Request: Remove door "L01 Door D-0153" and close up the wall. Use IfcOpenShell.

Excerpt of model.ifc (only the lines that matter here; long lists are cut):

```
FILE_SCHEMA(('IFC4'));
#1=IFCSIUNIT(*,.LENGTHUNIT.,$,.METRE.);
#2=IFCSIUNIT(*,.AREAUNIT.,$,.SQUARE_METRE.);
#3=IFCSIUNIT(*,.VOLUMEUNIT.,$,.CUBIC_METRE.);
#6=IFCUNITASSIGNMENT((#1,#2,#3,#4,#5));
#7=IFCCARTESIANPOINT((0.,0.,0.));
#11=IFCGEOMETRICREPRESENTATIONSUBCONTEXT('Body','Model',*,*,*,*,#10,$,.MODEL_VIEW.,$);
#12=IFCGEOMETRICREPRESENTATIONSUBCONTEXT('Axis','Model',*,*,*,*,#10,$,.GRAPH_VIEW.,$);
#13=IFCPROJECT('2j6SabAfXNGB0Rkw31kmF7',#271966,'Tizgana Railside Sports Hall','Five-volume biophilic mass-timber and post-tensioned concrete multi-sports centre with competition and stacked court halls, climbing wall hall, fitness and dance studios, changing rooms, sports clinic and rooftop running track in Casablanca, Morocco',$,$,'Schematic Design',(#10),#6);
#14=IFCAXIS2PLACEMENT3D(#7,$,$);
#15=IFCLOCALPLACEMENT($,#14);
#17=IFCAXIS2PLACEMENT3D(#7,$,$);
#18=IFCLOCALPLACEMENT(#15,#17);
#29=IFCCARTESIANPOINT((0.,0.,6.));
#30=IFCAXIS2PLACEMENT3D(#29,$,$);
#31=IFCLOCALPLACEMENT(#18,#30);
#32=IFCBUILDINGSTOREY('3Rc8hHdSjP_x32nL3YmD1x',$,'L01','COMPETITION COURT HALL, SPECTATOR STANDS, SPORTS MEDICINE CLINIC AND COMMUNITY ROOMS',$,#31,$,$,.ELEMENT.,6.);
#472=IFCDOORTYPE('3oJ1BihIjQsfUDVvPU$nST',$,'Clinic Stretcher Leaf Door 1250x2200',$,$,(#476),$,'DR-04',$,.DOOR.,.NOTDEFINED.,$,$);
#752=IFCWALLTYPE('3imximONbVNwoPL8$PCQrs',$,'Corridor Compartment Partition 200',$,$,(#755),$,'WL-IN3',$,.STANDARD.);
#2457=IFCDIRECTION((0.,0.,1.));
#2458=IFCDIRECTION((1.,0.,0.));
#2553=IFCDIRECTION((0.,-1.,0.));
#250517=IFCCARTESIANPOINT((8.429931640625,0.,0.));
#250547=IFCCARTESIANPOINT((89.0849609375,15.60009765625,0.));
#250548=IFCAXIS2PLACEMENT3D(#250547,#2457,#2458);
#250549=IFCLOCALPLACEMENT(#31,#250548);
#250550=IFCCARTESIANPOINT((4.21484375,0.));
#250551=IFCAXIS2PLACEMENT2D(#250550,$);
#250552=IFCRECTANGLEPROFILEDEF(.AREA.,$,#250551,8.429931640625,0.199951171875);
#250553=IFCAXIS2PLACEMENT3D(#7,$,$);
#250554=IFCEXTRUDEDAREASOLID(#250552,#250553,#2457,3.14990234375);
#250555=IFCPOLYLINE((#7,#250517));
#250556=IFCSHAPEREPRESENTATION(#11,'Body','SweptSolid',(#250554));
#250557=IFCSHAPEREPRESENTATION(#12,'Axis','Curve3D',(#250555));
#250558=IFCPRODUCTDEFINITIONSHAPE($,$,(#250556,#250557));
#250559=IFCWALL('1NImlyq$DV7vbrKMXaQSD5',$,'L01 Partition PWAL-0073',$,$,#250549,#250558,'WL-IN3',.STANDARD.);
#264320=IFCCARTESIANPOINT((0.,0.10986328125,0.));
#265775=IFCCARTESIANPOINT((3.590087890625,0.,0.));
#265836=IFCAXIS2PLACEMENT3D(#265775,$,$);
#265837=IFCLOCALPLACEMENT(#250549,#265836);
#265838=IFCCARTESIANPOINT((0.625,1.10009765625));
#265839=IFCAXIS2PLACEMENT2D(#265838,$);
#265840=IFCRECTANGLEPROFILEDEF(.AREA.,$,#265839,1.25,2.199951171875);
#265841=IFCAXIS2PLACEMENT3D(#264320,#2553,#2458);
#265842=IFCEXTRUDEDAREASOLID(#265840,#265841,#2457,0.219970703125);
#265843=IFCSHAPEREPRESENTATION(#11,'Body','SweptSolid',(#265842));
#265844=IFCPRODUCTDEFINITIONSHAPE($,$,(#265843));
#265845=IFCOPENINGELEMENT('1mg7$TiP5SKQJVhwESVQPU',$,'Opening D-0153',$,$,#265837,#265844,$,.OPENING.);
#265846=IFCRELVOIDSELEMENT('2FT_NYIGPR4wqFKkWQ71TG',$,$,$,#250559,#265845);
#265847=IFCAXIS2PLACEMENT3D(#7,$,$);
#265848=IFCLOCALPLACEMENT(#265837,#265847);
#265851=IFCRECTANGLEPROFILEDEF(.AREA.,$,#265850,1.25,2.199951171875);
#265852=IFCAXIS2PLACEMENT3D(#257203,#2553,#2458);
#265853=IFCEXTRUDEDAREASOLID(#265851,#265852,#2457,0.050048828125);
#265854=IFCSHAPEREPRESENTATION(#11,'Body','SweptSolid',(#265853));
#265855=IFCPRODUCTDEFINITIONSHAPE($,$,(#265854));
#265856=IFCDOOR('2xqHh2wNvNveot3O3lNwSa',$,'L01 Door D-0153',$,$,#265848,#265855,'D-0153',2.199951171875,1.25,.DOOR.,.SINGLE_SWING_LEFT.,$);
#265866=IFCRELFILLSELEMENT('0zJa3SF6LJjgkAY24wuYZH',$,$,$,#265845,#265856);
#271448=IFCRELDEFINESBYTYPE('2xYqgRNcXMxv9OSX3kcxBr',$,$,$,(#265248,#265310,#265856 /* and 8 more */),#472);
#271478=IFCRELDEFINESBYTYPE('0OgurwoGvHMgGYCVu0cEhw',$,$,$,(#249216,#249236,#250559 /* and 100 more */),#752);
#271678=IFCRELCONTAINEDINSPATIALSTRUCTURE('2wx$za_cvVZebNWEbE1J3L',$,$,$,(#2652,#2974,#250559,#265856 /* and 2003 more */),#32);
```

```python
import ifcopenshell
import ifcopenshell.api.feature
import ifcopenshell.api.root
import ifcopenshell.geom
import ifcopenshell.util.shape

model = ifcopenshell.open("model.ifc")
settings = ifcopenshell.geom.settings()


def volume(element):
    """Net volume in cubic metres, openings subtracted."""
    shape = ifcopenshell.geom.create_shape(settings, element)
    return ifcopenshell.util.shape.get_volume(shape.geometry)


door = model.by_id(265856)
opening = door.FillsVoids[0].RelatingOpeningElement
wall = opening.VoidsElements[0].RelatingBuildingElement
before = volume(wall)

ifcopenshell.api.root.remove_product(model, product=door)
ifcopenshell.api.feature.remove_feature(model, feature=opening)

after = volume(wall)

print(f"wall volume {before:.3f} -> {after:.3f} m3")

model.write("model_rev.ifc")
```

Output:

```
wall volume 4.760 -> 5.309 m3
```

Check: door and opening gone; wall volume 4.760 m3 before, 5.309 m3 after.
